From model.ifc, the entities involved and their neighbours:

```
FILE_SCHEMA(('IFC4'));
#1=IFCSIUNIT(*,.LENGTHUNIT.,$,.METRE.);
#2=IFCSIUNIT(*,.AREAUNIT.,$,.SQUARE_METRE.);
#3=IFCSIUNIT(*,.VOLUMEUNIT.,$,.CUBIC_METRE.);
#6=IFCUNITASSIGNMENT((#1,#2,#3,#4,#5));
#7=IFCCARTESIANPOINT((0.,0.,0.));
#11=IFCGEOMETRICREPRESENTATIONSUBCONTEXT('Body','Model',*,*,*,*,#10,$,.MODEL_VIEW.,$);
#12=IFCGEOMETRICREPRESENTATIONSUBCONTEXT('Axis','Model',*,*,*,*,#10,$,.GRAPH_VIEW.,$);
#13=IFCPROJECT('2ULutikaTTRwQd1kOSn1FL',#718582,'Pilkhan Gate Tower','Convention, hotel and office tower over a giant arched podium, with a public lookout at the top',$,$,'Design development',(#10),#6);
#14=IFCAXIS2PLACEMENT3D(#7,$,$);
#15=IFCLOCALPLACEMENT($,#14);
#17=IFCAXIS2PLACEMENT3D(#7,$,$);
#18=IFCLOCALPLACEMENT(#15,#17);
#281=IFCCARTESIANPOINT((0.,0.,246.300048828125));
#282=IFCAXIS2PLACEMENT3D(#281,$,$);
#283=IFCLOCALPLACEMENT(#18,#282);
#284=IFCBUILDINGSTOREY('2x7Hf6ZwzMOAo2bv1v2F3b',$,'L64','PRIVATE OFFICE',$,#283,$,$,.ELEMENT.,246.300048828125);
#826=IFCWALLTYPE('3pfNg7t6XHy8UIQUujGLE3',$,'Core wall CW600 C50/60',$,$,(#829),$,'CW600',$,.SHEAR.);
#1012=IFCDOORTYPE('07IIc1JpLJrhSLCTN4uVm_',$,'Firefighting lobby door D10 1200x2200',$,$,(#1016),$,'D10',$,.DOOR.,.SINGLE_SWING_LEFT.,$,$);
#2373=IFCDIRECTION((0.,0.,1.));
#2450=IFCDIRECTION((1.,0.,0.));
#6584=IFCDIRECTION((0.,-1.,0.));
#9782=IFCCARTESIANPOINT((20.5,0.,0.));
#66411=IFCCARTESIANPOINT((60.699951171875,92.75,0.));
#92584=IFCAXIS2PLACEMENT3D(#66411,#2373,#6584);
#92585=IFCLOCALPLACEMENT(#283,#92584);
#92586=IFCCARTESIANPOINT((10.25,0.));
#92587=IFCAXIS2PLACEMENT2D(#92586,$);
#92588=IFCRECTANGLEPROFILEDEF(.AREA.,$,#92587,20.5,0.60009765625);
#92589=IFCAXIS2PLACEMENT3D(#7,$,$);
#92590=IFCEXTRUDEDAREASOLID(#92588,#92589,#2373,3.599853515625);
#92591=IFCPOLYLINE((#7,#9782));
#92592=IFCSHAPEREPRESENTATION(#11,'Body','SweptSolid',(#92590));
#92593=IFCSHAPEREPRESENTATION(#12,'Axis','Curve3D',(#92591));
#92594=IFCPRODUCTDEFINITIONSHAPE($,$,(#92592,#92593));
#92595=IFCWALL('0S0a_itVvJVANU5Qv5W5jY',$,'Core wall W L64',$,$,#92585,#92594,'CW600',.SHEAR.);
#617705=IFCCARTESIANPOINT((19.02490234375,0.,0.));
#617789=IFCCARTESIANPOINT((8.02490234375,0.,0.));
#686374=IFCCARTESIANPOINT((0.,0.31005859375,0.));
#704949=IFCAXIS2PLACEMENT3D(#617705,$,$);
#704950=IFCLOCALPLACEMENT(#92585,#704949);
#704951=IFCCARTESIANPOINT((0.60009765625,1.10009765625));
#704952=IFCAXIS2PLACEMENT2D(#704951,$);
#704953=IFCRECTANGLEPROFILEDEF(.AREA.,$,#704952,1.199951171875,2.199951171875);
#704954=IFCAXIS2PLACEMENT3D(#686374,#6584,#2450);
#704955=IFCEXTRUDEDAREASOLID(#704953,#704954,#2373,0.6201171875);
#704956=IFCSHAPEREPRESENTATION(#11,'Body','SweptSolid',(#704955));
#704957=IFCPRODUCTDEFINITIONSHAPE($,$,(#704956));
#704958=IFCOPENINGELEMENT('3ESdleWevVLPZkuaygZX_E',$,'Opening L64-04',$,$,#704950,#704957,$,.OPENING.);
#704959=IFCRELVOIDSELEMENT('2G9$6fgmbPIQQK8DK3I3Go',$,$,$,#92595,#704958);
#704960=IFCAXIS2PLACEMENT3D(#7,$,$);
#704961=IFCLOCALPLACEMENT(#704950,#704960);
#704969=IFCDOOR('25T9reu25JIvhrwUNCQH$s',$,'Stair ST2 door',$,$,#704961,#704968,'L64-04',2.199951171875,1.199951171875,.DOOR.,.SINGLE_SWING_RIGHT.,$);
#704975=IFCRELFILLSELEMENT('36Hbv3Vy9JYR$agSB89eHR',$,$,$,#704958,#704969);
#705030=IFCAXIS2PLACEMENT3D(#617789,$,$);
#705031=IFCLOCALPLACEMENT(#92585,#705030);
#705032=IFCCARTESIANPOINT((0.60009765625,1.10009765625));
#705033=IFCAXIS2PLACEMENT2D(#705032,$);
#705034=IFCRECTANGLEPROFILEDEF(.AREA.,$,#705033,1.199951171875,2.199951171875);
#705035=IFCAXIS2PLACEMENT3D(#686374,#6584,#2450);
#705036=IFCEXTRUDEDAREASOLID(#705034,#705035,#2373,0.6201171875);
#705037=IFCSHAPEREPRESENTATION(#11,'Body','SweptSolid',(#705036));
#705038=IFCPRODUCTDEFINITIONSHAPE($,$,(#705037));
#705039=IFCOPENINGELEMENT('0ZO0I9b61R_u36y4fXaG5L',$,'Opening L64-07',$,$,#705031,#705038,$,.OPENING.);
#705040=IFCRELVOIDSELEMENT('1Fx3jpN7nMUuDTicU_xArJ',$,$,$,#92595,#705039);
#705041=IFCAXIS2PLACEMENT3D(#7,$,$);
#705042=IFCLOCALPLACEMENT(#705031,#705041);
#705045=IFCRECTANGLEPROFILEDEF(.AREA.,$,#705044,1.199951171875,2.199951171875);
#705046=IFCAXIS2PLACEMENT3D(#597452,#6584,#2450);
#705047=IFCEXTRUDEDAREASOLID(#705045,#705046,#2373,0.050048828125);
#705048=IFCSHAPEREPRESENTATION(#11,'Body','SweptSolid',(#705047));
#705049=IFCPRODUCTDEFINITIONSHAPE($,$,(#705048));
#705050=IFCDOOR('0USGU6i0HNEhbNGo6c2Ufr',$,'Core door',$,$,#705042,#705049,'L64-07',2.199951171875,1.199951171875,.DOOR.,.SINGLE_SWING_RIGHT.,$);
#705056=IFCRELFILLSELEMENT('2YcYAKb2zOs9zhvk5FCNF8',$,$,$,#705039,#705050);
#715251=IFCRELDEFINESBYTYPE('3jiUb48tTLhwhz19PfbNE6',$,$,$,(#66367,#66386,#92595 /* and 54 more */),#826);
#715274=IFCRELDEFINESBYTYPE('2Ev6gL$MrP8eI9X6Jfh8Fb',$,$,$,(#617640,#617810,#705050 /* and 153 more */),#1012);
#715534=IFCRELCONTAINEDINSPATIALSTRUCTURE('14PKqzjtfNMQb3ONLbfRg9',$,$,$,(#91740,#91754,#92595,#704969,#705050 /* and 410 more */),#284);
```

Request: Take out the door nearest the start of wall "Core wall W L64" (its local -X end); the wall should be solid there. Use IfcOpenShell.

```python
import ifcopenshell
import ifcopenshell.api.feature
import ifcopenshell.api.root
import ifcopenshell.geom
import ifcopenshell.util.shape

model = ifcopenshell.open("model.ifc")
settings = ifcopenshell.geom.settings()


def volume(element):
    """Net volume in cubic metres, openings subtracted."""
    shape = ifcopenshell.geom.create_shape(settings, element)
    return ifcopenshell.util.shape.get_volume(shape.geometry)


door = model.by_id(705050)
opening = door.FillsVoids[0].RelatingOpeningElement
wall = opening.VoidsElements[0].RelatingBuildingElement
before = volume(wall)

ifcopenshell.api.root.remove_product(model, product=door)
ifcopenshell.api.feature.remove_feature(model, feature=opening)

after = volume(wall)

print(f"wall volume {before:.3f} -> {after:.3f} m3")

model.write("model_edited.ifc")
```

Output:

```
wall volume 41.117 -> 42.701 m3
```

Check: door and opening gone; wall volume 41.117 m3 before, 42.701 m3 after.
